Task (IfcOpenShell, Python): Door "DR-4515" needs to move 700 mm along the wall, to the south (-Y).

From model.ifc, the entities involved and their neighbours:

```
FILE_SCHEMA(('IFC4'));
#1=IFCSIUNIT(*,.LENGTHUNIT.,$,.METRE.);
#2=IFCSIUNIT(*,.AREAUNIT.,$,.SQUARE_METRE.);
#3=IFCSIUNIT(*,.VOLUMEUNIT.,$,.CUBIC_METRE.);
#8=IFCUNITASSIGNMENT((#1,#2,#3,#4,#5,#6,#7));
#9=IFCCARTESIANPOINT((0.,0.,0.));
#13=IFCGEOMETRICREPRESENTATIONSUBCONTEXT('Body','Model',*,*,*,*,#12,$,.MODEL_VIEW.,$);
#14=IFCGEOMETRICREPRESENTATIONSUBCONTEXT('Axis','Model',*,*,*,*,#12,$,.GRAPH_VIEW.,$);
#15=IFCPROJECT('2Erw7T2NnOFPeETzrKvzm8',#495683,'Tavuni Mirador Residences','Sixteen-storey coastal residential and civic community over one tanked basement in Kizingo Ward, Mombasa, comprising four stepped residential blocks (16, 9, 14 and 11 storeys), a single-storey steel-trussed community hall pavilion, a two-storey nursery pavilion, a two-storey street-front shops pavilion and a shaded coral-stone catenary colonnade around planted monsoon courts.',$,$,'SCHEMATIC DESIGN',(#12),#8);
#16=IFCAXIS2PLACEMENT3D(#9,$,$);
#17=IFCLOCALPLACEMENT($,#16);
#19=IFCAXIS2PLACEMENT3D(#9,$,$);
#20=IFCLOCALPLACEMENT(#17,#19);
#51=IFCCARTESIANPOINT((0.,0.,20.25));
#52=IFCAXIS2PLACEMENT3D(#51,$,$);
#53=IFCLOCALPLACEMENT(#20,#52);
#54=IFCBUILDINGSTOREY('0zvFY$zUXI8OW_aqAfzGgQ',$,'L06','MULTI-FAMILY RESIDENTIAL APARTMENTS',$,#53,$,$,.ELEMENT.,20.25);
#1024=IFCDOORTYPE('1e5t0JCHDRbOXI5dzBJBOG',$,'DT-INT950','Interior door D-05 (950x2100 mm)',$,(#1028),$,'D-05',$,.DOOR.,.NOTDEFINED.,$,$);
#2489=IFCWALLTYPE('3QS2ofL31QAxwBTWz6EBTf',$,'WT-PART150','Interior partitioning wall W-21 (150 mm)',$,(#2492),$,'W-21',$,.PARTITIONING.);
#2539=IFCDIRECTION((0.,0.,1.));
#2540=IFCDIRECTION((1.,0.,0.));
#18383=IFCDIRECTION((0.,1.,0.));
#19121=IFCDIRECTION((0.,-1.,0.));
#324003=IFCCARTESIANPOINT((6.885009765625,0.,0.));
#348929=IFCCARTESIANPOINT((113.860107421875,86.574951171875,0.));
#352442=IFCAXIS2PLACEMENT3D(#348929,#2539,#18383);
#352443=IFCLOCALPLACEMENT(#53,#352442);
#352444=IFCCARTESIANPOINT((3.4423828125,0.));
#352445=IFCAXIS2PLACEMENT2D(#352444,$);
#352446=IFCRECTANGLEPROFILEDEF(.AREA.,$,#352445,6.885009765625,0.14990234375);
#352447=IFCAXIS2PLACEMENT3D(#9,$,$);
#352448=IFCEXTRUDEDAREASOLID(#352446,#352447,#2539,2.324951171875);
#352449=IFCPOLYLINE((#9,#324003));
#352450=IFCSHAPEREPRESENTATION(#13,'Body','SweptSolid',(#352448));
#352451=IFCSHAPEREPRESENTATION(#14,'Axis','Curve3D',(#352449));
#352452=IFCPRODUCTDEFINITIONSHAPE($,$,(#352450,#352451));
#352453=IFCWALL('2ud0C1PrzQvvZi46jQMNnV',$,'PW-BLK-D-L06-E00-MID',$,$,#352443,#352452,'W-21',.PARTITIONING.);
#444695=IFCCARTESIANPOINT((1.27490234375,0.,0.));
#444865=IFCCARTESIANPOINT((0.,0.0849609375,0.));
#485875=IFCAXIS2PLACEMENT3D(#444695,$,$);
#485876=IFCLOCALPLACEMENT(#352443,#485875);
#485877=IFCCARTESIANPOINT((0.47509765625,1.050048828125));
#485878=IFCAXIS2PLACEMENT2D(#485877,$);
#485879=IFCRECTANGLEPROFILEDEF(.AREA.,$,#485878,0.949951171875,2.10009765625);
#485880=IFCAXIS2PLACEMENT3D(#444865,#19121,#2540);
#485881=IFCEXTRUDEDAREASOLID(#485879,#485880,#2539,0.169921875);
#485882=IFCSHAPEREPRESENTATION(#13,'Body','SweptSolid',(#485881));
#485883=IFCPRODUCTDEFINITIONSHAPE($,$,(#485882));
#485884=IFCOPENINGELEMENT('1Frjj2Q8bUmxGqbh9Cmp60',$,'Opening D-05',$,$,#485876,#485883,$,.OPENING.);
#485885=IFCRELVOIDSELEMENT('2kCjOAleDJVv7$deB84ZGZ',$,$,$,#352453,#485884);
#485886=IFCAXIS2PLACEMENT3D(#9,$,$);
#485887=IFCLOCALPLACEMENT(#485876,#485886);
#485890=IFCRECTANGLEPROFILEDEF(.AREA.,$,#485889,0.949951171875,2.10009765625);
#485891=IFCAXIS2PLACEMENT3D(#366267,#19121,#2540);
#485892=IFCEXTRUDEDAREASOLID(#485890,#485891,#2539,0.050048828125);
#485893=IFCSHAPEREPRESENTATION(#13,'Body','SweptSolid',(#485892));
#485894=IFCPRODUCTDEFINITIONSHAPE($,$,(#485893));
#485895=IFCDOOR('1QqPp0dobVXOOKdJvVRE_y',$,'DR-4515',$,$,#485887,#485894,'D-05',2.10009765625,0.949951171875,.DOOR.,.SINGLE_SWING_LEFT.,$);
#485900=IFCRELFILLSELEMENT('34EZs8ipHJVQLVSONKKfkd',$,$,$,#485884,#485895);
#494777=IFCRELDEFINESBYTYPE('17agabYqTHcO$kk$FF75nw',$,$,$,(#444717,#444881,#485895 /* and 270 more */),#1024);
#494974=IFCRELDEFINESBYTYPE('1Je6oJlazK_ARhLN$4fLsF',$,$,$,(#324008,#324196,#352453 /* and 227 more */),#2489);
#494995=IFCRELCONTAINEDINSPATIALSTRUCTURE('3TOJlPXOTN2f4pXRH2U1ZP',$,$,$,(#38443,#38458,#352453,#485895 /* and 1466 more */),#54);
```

```python
import ifcopenshell
import ifcopenshell.api.geometry
import ifcopenshell.util.placement
import ifcopenshell.util.unit

model = ifcopenshell.open("model.ifc")
unit_scale = ifcopenshell.util.unit.calculate_unit_scale(model)

door = model.by_guid("1QqPp0dobVXOOKdJvVRE_y")
opening = door.FillsVoids[0].RelatingOpeningElement
wall = opening.VoidsElements[0].RelatingBuildingElement

wall_matrix = ifcopenshell.util.placement.get_local_placement(wall.ObjectPlacement)
shift = wall_matrix[:3, 0] * -0.7 / unit_scale
before = ifcopenshell.util.placement.get_local_placement(door.ObjectPlacement)[:3, 3].copy()

# The door is placed relative to its opening, so it follows when the opening moves.
matrix = ifcopenshell.util.placement.get_local_placement(opening.ObjectPlacement)
matrix[:3, 3] += shift
ifcopenshell.api.geometry.edit_object_placement(
    model, product=opening, matrix=matrix, is_si=False, should_transform_children=True
)

after = ifcopenshell.util.placement.get_local_placement(door.ObjectPlacement)[:3, 3]
print("door moved by", (after - before).round(3) + 0.0)

model.write("model-out.ifc")
```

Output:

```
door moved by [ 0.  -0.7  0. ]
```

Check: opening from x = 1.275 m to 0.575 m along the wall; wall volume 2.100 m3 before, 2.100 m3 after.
